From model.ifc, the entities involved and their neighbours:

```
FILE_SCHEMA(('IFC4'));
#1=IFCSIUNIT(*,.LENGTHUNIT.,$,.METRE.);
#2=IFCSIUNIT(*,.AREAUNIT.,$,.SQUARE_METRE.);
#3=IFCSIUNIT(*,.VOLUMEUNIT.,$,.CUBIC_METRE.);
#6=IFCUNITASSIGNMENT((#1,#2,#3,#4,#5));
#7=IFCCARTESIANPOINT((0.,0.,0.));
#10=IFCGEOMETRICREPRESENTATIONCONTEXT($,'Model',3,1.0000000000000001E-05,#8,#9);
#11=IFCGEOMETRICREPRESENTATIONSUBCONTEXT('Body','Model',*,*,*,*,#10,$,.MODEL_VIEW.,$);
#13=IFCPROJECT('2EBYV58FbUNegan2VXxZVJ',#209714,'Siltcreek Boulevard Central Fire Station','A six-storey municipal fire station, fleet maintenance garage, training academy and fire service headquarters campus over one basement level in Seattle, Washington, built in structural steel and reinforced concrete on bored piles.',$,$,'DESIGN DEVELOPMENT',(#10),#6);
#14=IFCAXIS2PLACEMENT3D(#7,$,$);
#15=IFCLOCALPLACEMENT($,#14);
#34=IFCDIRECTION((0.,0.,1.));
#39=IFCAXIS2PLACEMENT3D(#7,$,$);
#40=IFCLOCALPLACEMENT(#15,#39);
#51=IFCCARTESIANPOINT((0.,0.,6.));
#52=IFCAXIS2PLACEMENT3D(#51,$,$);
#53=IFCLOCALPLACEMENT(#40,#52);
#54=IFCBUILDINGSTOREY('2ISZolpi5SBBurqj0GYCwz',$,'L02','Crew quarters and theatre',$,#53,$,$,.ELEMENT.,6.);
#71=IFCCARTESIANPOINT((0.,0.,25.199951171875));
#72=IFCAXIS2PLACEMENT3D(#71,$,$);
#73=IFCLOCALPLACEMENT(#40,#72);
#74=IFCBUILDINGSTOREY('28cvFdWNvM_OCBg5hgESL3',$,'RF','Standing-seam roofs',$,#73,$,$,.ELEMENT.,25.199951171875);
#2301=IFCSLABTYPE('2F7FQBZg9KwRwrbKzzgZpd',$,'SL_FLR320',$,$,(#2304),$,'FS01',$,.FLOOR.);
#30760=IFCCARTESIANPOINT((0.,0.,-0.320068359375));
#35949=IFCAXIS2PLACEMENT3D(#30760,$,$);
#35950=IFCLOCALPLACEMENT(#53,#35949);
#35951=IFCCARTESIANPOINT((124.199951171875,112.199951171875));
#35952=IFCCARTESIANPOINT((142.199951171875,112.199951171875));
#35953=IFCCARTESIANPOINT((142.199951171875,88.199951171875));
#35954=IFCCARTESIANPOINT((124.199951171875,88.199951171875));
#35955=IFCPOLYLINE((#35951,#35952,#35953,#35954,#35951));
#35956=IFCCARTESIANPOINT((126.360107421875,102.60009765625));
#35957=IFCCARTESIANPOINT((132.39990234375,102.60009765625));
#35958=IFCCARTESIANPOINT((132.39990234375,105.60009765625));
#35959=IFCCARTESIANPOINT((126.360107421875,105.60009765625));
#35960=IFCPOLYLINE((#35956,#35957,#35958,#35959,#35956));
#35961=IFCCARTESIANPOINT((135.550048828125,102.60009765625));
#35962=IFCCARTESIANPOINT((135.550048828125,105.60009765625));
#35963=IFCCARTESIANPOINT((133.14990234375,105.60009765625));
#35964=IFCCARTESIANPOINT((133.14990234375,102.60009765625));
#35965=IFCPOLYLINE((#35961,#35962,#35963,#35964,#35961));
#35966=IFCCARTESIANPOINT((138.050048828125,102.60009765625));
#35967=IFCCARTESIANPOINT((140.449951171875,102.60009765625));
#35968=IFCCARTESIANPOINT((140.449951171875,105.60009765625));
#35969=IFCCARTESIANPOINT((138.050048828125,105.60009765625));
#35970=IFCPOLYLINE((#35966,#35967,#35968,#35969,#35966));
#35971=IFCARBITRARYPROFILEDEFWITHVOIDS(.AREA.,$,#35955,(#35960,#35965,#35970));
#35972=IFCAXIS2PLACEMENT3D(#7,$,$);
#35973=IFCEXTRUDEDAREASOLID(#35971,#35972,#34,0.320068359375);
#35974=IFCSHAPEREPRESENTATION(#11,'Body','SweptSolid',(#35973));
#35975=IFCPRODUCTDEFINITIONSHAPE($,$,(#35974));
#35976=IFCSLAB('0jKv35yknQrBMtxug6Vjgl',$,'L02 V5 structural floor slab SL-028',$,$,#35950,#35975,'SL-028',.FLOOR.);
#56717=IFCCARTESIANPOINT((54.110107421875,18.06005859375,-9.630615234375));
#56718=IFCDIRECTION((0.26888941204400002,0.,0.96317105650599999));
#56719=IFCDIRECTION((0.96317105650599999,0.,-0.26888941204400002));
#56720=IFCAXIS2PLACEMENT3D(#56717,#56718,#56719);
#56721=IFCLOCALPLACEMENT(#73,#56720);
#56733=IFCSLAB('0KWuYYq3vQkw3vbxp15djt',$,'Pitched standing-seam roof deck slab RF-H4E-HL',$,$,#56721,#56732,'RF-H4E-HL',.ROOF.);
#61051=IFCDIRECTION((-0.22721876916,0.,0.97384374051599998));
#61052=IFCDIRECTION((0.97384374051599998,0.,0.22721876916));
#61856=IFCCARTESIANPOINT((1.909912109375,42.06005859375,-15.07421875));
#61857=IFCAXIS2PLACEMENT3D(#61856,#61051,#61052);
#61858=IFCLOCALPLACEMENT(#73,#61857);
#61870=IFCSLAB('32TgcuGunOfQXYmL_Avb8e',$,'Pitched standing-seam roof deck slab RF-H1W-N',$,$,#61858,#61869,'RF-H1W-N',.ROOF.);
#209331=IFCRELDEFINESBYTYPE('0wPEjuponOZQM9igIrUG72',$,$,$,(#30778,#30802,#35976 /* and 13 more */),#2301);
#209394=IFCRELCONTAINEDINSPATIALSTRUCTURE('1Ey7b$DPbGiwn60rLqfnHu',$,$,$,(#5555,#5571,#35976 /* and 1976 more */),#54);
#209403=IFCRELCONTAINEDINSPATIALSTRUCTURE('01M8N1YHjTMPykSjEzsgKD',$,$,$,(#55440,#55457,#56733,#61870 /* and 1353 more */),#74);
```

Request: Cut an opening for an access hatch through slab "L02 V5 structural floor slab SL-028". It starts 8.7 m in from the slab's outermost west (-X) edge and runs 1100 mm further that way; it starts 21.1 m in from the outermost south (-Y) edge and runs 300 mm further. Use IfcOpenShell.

```python
import numpy as np
import ifcopenshell
import ifcopenshell.api.feature
import ifcopenshell.api.geometry
import ifcopenshell.api.root
import ifcopenshell.geom
import ifcopenshell.util.placement
import ifcopenshell.util.representation
import ifcopenshell.util.shape
import ifcopenshell.util.unit

model = ifcopenshell.open("model.ifc")
unit_scale = ifcopenshell.util.unit.calculate_unit_scale(model)
settings = ifcopenshell.geom.settings()


def volume(element):
    """Net volume in cubic metres, openings subtracted."""
    shape = ifcopenshell.geom.create_shape(settings, element)
    return ifcopenshell.util.shape.get_volume(shape.geometry)


slab = model.by_guid("0jKv35yknQrBMtxug6Vjgl")
before = volume(slab)

# Extent in the slab's own axes, in metres. The edges named are its -X and -Y sides.
slab_shape = ifcopenshell.geom.create_shape(settings, slab)
vertices = ifcopenshell.util.shape.get_vertices(slab_shape.geometry)
x_min, y_min, bottom = vertices.min(axis=0)
top = vertices[:, 2].max()

opening = ifcopenshell.api.root.create_entity(model, ifc_class="IfcOpeningElement", name="Access hatch opening", predefined_type="OPENING")
context = ifcopenshell.util.representation.get_context(model, "Model", "Body", "MODEL_VIEW")
width, depth = 1.1, 0.3
outline = [(0.0, 0.0), (width, 0.0), (width, depth), (0.0, depth), (0.0, 0.0)]
# Overshoot both faces by 50 mm so the cut is clean.
shape = ifcopenshell.api.geometry.add_slab_representation(
    model, context=context, depth=top - bottom + 0.1, polyline=outline
)
ifcopenshell.api.geometry.assign_representation(model, product=opening, representation=shape)

matrix = ifcopenshell.util.placement.get_local_placement(slab.ObjectPlacement)
matrix[:, 3] = matrix @ np.append(np.array([x_min + 8.7, y_min + 21.1, bottom - 0.05]) / unit_scale, 1.0)
ifcopenshell.api.geometry.edit_object_placement(model, product=opening, matrix=matrix, is_si=False)
ifcopenshell.api.feature.add_feature(model, feature=opening, element=slab)

after = volume(slab)

print(f"slab volume {before:.3f} -> {after:.3f} m3")

model.write("model-out.ifc")
```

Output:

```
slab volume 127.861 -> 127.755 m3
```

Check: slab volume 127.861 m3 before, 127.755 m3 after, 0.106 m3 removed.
